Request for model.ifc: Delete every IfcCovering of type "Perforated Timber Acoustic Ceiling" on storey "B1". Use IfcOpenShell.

First a look at what the model holds.

```python
import ifcopenshell
import ifcopenshell.util.element

model = ifcopenshell.open("model.ifc")
print(model.schema)
storey = next(s for s in model.by_type("IfcBuildingStorey") if s.Name == "B1")
coverings = [e for e in ifcopenshell.util.element.get_decomposition(storey) if e.is_a("IfcCovering")]
seen = {}
for e in coverings:
    element_type = ifcopenshell.util.element.get_type(e)
    name = element_type.Name if element_type not in (None, e) else None
    seen[name] = seen.get(name, 0) + 1
for name, count in sorted(seen.items(), key=str):
    print(count, "x", name)
```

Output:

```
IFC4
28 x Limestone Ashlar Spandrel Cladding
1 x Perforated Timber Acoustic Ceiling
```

```python
import ifcopenshell
import ifcopenshell.api.root
import ifcopenshell.util.element

model = ifcopenshell.open("model.ifc")

storey = next(s for s in model.by_type("IfcBuildingStorey") if s.Name == "B1")
coverings = [e for e in ifcopenshell.util.element.get_decomposition(storey) if e.is_a("IfcCovering")]
targets = [e for e in coverings if (t := ifcopenshell.util.element.get_type(e)) not in (None, e) and t.Name == "Perforated Timber Acoustic Ceiling"]

for e in targets:
    ifcopenshell.api.root.remove_product(model, product=e)
print(len(targets), "removed")

model.write("model_rev.ifc")
```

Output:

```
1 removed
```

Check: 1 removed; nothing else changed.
